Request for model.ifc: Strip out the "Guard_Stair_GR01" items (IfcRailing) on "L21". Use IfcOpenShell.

First a look at what the model holds.

```python
import ifcopenshell
import ifcopenshell.util.element

model = ifcopenshell.open("model.ifc")
print(model.schema)
storey = next(s for s in model.by_type("IfcBuildingStorey") if s.Name == "L21")
railings = [e for e in ifcopenshell.util.element.get_decomposition(storey) if e.is_a("IfcRailing")]
seen = {}
for e in railings:
    element_type = ifcopenshell.util.element.get_type(e)
    name = element_type.Name if element_type not in (None, e) else None
    seen[name] = seen.get(name, 0) + 1
for name, count in sorted(seen.items(), key=str):
    print(count, "x", name)
```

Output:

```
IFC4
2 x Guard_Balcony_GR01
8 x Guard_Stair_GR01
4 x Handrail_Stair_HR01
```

```python
import ifcopenshell
import ifcopenshell.api.root
import ifcopenshell.util.element

model = ifcopenshell.open("model.ifc")

storey = next(s for s in model.by_type("IfcBuildingStorey") if s.Name == "L21")
railings = [e for e in ifcopenshell.util.element.get_decomposition(storey) if e.is_a("IfcRailing")]
targets = [e for e in railings if (t := ifcopenshell.util.element.get_type(e)) not in (None, e) and t.Name == "Guard_Stair_GR01"]

for e in targets:
    ifcopenshell.api.root.remove_product(model, product=e)
print(len(targets), "removed")

model.write("model-out.ifc")
```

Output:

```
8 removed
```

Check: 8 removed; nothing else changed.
